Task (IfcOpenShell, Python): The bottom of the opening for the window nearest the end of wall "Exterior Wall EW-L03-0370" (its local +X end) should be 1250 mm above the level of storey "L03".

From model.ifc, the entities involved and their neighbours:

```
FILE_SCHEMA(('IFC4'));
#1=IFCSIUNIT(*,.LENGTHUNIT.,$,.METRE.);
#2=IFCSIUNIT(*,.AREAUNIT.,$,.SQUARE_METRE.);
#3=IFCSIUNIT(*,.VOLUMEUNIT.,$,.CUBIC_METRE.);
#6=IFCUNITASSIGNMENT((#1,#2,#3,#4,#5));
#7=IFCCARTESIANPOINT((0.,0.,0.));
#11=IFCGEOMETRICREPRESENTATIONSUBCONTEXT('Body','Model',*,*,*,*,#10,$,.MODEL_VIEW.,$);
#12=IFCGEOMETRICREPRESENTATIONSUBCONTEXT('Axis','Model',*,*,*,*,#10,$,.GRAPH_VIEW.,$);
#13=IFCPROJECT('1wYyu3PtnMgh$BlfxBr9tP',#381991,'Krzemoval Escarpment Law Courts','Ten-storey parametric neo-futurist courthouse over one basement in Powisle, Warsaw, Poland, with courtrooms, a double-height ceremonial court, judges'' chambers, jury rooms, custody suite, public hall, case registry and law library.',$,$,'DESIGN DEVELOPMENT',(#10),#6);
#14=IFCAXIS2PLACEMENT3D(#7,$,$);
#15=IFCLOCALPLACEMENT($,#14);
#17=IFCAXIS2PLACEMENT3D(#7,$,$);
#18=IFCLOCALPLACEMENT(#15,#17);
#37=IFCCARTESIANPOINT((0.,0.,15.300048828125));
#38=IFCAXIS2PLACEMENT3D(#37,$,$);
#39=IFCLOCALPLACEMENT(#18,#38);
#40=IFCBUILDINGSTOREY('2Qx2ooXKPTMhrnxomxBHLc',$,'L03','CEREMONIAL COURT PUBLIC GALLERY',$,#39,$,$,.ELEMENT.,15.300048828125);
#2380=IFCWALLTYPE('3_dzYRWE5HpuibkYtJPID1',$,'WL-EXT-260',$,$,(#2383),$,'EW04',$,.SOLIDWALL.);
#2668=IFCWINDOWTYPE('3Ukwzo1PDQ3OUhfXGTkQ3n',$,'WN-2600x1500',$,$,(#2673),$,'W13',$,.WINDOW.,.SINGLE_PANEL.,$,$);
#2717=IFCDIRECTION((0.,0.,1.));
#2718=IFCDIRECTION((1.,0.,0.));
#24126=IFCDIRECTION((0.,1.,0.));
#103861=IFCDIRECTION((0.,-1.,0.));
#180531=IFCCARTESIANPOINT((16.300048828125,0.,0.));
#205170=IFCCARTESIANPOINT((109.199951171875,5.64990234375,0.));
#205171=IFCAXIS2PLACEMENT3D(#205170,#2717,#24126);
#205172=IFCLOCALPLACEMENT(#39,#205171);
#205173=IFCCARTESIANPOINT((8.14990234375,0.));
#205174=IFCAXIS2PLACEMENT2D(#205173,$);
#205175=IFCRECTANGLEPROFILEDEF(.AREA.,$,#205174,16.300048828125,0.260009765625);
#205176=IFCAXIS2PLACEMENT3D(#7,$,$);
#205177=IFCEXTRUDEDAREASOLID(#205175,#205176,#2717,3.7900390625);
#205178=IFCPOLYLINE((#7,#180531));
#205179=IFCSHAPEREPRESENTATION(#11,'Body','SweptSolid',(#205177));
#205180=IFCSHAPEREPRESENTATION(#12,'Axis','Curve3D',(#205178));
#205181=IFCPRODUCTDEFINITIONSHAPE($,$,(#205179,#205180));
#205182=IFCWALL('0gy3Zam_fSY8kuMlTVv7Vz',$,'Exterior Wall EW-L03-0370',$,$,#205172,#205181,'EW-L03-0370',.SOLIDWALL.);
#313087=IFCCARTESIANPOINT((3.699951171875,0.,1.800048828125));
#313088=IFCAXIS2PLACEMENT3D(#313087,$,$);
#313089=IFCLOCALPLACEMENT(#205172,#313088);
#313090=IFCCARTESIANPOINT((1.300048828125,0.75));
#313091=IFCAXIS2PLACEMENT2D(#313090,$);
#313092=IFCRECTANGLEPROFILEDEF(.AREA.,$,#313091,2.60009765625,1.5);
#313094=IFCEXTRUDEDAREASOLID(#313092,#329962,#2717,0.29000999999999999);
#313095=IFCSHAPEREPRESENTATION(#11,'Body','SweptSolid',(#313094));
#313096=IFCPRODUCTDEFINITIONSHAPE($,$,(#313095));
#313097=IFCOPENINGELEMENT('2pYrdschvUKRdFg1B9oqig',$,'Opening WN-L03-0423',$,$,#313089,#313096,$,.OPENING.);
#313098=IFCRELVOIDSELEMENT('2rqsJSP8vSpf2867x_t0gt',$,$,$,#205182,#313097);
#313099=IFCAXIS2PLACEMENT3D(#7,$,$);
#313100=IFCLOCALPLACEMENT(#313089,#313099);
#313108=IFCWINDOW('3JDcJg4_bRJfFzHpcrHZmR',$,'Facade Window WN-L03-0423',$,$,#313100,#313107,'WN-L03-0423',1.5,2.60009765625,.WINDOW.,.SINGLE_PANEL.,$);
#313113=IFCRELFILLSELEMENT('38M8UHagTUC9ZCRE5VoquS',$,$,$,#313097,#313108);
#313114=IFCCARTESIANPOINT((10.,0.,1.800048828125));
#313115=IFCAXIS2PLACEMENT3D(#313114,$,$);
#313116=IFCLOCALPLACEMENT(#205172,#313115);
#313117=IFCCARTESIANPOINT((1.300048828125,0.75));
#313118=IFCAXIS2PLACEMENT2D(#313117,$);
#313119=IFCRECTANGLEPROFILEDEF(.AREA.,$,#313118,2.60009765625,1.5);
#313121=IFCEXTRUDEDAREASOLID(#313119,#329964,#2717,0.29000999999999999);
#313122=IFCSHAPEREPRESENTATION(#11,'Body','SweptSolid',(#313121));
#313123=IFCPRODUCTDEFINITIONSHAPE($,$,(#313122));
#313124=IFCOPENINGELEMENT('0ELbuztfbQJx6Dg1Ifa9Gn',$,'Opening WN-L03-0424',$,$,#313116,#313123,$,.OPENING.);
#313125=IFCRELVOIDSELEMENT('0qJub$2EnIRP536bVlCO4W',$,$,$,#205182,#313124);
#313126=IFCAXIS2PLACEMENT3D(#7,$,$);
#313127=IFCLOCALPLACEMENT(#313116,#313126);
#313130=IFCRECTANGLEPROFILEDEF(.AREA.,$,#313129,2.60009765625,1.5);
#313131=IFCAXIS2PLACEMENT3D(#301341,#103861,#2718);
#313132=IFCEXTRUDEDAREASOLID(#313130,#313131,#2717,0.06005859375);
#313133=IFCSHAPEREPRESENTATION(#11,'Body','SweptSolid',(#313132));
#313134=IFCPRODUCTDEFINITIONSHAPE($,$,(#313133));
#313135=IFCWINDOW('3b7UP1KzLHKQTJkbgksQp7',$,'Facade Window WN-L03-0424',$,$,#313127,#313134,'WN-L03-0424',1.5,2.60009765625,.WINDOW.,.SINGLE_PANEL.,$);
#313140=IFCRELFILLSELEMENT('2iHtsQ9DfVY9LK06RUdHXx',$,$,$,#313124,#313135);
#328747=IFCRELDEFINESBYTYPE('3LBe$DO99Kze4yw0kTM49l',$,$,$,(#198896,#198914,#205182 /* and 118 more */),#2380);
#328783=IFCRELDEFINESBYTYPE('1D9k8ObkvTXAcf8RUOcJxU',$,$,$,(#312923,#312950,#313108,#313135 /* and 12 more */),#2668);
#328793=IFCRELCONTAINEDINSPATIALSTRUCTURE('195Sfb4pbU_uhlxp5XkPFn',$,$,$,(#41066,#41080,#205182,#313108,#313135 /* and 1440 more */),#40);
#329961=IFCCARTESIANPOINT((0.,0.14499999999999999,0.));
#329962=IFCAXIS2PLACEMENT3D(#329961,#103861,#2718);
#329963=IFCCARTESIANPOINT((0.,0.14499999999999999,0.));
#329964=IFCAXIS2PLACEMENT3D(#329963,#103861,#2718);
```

```python
import numpy as np
import ifcopenshell
import ifcopenshell.api.geometry
import ifcopenshell.geom
import ifcopenshell.util.element
import ifcopenshell.util.placement
import ifcopenshell.util.shape
import ifcopenshell.util.unit

model = ifcopenshell.open("model.ifc")
unit_scale = ifcopenshell.util.unit.calculate_unit_scale(model)

window = model.by_id(313135)
opening = window.FillsVoids[0].RelatingOpeningElement
storey = ifcopenshell.util.element.get_container(window, ifc_class="IfcBuildingStorey")
level = ifcopenshell.util.placement.get_local_placement(storey.ObjectPlacement)[2, 3]

# The opening's origin need not be at the sill, so measure its lowest point.
shape = ifcopenshell.geom.create_shape(ifcopenshell.geom.settings(), opening)
bottom = ifcopenshell.util.shape.get_shape_bottom_elevation(shape, shape.geometry) / unit_scale
dz = level + 1.25 - bottom

shift = np.array([0.0, 0.0, dz])
# The window is placed relative to its opening, so it follows when the opening moves.
matrix = ifcopenshell.util.placement.get_local_placement(opening.ObjectPlacement)
matrix[:3, 3] += shift
ifcopenshell.api.geometry.edit_object_placement(
    model, product=opening, matrix=matrix, is_si=False, should_transform_children=True
)

print(f"moved by {dz * unit_scale:+.3f} m")

model.write("model_edited.ifc")
```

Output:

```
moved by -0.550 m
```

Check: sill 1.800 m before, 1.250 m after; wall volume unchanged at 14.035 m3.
